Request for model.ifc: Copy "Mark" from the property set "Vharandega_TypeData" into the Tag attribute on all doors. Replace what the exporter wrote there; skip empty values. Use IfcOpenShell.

First a look at what the model holds.

```python
import ifcopenshell
import ifcopenshell.util.element

model = ifcopenshell.open("model.ifc")
print(model.schema)
doors = model.by_type("IfcDoor")
print(len(doors), "doors")
for e in doors[:8]:
    source = ifcopenshell.util.element.get_pset(e, "Vharandega_TypeData", "Mark")
    target = e.Tag
    print(e.id(), repr(source), repr(target), sep=" | ")
```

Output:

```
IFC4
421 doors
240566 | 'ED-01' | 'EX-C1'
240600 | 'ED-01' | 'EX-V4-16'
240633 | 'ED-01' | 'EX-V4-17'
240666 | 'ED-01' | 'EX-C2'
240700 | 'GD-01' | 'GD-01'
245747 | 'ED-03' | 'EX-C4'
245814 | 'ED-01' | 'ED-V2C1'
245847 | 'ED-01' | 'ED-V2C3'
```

```python
import ifcopenshell
import ifcopenshell.util.element

model = ifcopenshell.open("model.ifc")

count = 0
for e in model.by_type("IfcDoor"):
    value = ifcopenshell.util.element.get_pset(e, "Vharandega_TypeData", "Mark")
    current = e.Tag
    if not value or not value.strip() or current == value:
        continue
    e.Tag = value
    count += 1

print(count, "doors updated")

model.write("model_v2.ifc")
```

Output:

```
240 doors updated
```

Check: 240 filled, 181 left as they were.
